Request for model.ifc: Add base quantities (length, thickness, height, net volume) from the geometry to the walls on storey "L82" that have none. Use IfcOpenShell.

First a look at what the model holds.

```python
import ifcopenshell
import ifcopenshell.util.element
import ifcopenshell.util.unit

model = ifcopenshell.open("model.ifc")
print(model.schema)
for unit_type in ("LENGTHUNIT", "AREAUNIT", "VOLUMEUNIT"):
    print(unit_type, ifcopenshell.util.unit.calculate_unit_scale(model, unit_type))
storey = next(s for s in model.by_type("IfcBuildingStorey") if s.Name == "L82")
walls = [e for e in ifcopenshell.util.element.get_decomposition(storey) if e.is_a("IfcWall")]
for e in sorted(walls, key=lambda e: e.id()):
    print(e.id(), e.is_a(), e.Name, list(ifcopenshell.util.element.get_psets(e, qtos_only=True)), sep=" | ")
```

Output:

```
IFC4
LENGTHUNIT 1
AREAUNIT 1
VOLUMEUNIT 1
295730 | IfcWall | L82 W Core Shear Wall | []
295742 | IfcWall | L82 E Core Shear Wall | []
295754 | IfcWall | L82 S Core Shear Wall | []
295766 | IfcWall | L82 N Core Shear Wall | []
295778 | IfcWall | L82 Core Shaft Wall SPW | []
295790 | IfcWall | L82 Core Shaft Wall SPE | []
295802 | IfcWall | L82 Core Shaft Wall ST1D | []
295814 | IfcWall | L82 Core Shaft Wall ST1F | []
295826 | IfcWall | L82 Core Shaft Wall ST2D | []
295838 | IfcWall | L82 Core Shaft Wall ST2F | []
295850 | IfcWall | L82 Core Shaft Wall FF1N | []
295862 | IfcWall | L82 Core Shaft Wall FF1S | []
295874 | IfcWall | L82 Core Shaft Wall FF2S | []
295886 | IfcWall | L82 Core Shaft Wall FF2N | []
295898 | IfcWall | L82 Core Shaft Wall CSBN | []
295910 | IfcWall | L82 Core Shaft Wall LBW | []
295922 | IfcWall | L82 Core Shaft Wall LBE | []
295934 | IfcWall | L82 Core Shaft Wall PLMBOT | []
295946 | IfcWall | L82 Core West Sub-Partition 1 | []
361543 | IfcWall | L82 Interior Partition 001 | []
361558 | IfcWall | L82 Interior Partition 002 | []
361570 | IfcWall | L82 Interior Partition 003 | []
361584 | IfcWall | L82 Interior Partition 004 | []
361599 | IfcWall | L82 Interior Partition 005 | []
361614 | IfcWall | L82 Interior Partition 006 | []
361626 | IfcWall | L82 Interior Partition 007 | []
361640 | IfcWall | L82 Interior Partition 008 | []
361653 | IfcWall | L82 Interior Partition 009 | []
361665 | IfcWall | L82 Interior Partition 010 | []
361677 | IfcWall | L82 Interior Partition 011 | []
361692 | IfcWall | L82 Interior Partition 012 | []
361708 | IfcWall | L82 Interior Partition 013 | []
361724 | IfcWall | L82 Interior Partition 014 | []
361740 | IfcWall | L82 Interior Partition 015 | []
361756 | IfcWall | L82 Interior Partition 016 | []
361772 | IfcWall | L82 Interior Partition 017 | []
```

```python
import ifcopenshell
import ifcopenshell.api.pset
import ifcopenshell.geom
import ifcopenshell.util.element
import ifcopenshell.util.shape
import ifcopenshell.util.unit

model = ifcopenshell.open("model.ifc")
unit_scale = ifcopenshell.util.unit.calculate_unit_scale(model)
volume_scale = ifcopenshell.util.unit.calculate_unit_scale(model, "VOLUMEUNIT")
settings = ifcopenshell.geom.settings()

storey = next(s for s in model.by_type("IfcBuildingStorey") if s.Name == "L82")
walls = [e for e in ifcopenshell.util.element.get_decomposition(storey) if e.is_a("IfcWall")]

for e in sorted(walls, key=lambda e: e.id()):
    if ifcopenshell.util.element.get_psets(e, qtos_only=True, should_inherit=False):
        continue
    # Geometry comes back in metres, in the element's own axes.
    shape = ifcopenshell.geom.create_shape(settings, e)
    values = {
        "Length": ifcopenshell.util.shape.get_x(shape.geometry) / unit_scale,
        "Width": ifcopenshell.util.shape.get_y(shape.geometry) / unit_scale,
        "Height": ifcopenshell.util.shape.get_z(shape.geometry) / unit_scale,
        "NetVolume": ifcopenshell.util.shape.get_volume(shape.geometry) / volume_scale,
    }
    qto = ifcopenshell.api.pset.add_qto(model, product=e, name="Qto_WallBaseQuantities")
    ifcopenshell.api.pset.edit_qto(model, qto=qto, properties=values)
    print(e.id(), {k: round(v, 3) for k, v in values.items()})

model.write("model_rev.ifc")
```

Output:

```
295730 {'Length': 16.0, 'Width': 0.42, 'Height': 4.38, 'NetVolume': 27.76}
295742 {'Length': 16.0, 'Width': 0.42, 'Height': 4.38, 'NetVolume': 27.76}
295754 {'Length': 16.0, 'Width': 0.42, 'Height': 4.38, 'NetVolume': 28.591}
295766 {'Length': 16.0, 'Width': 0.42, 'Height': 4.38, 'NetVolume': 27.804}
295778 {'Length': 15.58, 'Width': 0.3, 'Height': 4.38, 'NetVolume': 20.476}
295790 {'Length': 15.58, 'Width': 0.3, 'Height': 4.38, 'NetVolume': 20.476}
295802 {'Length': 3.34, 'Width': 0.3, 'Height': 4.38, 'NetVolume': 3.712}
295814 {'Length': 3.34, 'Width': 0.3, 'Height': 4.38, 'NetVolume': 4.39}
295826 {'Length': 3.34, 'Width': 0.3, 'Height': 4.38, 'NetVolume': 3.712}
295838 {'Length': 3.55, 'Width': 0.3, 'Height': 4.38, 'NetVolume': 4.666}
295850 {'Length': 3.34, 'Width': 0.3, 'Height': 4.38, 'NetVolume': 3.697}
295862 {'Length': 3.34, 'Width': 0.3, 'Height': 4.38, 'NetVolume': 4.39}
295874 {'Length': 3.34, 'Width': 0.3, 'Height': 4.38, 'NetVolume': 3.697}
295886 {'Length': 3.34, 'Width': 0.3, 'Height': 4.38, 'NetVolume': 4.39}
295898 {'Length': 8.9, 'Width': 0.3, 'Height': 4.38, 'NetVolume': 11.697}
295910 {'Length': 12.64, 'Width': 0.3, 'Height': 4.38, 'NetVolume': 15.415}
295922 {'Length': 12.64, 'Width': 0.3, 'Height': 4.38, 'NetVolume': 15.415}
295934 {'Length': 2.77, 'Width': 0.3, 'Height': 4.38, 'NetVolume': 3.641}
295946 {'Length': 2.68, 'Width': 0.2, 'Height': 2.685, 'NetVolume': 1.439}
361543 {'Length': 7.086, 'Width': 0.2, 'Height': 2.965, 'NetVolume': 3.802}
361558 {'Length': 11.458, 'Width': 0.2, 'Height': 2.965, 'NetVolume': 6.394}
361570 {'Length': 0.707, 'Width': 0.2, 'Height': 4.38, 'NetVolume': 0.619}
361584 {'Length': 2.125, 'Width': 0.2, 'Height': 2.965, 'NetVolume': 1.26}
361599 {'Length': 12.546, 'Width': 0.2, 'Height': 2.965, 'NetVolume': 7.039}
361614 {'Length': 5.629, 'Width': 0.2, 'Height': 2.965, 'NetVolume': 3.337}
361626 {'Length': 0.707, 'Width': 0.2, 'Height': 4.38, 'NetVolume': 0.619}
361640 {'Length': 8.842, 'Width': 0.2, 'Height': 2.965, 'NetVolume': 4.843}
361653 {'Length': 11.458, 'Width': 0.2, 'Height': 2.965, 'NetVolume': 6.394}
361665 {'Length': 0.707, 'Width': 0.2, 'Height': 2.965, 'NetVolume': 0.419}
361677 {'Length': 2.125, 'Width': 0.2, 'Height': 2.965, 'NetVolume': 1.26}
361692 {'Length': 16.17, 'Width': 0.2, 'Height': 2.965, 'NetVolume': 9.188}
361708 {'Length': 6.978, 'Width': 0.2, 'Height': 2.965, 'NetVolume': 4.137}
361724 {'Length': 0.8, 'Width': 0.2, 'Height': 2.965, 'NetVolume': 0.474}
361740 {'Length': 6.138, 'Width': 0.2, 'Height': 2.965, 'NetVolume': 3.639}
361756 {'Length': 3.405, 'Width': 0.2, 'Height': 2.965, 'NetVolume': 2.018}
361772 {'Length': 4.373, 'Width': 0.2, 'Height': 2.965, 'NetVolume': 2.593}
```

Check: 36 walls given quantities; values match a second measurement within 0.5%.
